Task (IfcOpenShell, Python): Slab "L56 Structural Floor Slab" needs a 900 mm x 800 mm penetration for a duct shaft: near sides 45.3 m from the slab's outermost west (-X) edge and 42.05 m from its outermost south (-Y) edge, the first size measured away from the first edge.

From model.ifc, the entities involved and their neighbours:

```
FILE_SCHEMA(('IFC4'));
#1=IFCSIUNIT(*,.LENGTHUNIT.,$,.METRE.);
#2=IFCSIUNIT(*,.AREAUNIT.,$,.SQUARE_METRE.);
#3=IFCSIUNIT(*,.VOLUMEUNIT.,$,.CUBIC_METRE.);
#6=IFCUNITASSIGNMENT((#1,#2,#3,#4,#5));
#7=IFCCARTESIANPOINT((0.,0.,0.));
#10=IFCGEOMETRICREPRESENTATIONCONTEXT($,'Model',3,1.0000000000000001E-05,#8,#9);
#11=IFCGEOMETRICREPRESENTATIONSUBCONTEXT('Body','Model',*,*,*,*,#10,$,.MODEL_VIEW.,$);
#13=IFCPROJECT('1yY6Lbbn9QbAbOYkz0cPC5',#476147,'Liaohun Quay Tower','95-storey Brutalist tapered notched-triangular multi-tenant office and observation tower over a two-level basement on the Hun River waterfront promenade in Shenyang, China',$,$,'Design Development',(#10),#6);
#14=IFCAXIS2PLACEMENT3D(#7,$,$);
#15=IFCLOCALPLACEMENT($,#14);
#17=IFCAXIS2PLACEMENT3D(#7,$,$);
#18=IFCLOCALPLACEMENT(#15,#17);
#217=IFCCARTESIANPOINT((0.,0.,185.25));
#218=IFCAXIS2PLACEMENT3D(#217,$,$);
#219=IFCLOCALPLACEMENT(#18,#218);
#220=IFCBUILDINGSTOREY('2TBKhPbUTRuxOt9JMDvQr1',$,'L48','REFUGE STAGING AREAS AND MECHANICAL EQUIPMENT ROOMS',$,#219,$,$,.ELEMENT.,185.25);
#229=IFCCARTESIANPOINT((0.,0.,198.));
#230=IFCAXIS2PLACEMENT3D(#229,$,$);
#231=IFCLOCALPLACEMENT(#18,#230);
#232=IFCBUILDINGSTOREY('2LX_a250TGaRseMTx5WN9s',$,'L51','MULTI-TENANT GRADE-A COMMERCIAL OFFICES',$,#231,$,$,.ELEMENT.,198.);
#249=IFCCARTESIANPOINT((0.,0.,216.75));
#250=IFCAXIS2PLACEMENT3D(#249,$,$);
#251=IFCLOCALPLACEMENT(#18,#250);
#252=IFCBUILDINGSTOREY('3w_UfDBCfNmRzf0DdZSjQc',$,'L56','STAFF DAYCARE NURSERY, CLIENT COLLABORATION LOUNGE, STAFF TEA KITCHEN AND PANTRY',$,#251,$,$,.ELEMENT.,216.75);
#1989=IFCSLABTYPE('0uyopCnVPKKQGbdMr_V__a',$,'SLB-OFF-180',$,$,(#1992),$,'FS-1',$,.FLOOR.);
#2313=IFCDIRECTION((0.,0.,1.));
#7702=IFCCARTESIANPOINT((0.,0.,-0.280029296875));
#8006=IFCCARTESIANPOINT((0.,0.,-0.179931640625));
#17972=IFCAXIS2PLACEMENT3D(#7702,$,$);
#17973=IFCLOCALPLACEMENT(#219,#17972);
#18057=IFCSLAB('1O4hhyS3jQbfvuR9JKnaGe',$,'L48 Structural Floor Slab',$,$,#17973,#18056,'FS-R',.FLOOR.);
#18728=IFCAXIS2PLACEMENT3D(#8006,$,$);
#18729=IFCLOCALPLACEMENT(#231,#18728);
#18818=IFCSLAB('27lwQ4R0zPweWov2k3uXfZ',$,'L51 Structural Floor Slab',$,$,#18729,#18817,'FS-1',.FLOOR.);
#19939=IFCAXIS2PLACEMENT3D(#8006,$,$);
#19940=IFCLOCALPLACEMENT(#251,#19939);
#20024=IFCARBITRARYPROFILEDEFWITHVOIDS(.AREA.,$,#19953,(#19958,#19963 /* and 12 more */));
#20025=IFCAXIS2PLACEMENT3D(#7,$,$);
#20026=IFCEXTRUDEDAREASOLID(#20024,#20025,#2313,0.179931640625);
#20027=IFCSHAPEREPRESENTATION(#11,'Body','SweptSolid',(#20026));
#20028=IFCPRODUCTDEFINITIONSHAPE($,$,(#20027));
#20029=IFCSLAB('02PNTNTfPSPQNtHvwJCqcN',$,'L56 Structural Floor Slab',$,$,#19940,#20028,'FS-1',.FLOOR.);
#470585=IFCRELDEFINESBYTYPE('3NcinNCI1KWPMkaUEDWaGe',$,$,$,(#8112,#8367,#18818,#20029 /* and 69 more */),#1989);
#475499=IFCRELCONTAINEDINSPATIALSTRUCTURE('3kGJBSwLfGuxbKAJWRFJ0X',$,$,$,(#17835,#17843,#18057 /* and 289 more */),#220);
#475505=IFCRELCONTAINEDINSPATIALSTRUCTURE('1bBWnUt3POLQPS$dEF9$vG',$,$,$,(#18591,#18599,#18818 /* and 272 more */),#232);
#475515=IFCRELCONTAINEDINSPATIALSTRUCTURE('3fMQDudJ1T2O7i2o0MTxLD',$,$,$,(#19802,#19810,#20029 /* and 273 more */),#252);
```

```python
import numpy as np
import ifcopenshell
import ifcopenshell.api.feature
import ifcopenshell.api.geometry
import ifcopenshell.api.root
import ifcopenshell.geom
import ifcopenshell.util.placement
import ifcopenshell.util.representation
import ifcopenshell.util.shape
import ifcopenshell.util.unit

model = ifcopenshell.open("model.ifc")
unit_scale = ifcopenshell.util.unit.calculate_unit_scale(model)
settings = ifcopenshell.geom.settings()


def volume(element):
    """Net volume in cubic metres, openings subtracted."""
    shape = ifcopenshell.geom.create_shape(settings, element)
    return ifcopenshell.util.shape.get_volume(shape.geometry)


slab = model.by_id(20029)
before = volume(slab)

# Extent in the slab's own axes, in metres. The edges named are its -X and -Y sides.
slab_shape = ifcopenshell.geom.create_shape(settings, slab)
vertices = ifcopenshell.util.shape.get_vertices(slab_shape.geometry)
x_min, y_min, bottom = vertices.min(axis=0)
top = vertices[:, 2].max()

opening = ifcopenshell.api.root.create_entity(model, ifc_class="IfcOpeningElement", name="Duct shaft opening", predefined_type="OPENING")
context = ifcopenshell.util.representation.get_context(model, "Model", "Body", "MODEL_VIEW")
width, depth = 0.9, 0.8
outline = [(0.0, 0.0), (width, 0.0), (width, depth), (0.0, depth), (0.0, 0.0)]
# Overshoot both faces by 50 mm so the cut is clean.
shape = ifcopenshell.api.geometry.add_slab_representation(
    model, context=context, depth=top - bottom + 0.1, polyline=outline
)
ifcopenshell.api.geometry.assign_representation(model, product=opening, representation=shape)

matrix = ifcopenshell.util.placement.get_local_placement(slab.ObjectPlacement)
matrix[:, 3] = matrix @ np.append(np.array([x_min + 45.3, y_min + 42.05, bottom - 0.05]) / unit_scale, 1.0)
ifcopenshell.api.geometry.edit_object_placement(model, product=opening, matrix=matrix, is_si=False)
ifcopenshell.api.feature.add_feature(model, feature=opening, element=slab)

after = volume(slab)

print(f"slab volume {before:.3f} -> {after:.3f} m3")

model.write("model_v2.ifc")
```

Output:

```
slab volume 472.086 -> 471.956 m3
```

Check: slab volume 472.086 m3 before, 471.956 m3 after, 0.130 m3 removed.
